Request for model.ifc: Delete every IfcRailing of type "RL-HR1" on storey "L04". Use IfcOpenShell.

First a look at what the model holds.

```python
import ifcopenshell
import ifcopenshell.util.element

model = ifcopenshell.open("model.ifc")
print(model.schema)
storey = next(s for s in model.by_type("IfcBuildingStorey") if s.Name == "L04")
railings = [e for e in ifcopenshell.util.element.get_decomposition(storey) if e.is_a("IfcRailing")]
seen = {}
for e in railings:
    element_type = ifcopenshell.util.element.get_type(e)
    name = element_type.Name if element_type not in (None, e) else None
    seen[name] = seen.get(name, 0) + 1
for name, count in sorted(seen.items(), key=str):
    print(count, "x", name)
```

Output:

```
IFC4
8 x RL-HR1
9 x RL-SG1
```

```python
import ifcopenshell
import ifcopenshell.api.root
import ifcopenshell.util.element

model = ifcopenshell.open("model.ifc")

storey = next(s for s in model.by_type("IfcBuildingStorey") if s.Name == "L04")
railings = [e for e in ifcopenshell.util.element.get_decomposition(storey) if e.is_a("IfcRailing")]
targets = [e for e in railings if (t := ifcopenshell.util.element.get_type(e)) not in (None, e) and t.Name == "RL-HR1"]

for e in targets:
    ifcopenshell.api.root.remove_product(model, product=e)
print(len(targets), "removed")

model.write("model_rev.ifc")
```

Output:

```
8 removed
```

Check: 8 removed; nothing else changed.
